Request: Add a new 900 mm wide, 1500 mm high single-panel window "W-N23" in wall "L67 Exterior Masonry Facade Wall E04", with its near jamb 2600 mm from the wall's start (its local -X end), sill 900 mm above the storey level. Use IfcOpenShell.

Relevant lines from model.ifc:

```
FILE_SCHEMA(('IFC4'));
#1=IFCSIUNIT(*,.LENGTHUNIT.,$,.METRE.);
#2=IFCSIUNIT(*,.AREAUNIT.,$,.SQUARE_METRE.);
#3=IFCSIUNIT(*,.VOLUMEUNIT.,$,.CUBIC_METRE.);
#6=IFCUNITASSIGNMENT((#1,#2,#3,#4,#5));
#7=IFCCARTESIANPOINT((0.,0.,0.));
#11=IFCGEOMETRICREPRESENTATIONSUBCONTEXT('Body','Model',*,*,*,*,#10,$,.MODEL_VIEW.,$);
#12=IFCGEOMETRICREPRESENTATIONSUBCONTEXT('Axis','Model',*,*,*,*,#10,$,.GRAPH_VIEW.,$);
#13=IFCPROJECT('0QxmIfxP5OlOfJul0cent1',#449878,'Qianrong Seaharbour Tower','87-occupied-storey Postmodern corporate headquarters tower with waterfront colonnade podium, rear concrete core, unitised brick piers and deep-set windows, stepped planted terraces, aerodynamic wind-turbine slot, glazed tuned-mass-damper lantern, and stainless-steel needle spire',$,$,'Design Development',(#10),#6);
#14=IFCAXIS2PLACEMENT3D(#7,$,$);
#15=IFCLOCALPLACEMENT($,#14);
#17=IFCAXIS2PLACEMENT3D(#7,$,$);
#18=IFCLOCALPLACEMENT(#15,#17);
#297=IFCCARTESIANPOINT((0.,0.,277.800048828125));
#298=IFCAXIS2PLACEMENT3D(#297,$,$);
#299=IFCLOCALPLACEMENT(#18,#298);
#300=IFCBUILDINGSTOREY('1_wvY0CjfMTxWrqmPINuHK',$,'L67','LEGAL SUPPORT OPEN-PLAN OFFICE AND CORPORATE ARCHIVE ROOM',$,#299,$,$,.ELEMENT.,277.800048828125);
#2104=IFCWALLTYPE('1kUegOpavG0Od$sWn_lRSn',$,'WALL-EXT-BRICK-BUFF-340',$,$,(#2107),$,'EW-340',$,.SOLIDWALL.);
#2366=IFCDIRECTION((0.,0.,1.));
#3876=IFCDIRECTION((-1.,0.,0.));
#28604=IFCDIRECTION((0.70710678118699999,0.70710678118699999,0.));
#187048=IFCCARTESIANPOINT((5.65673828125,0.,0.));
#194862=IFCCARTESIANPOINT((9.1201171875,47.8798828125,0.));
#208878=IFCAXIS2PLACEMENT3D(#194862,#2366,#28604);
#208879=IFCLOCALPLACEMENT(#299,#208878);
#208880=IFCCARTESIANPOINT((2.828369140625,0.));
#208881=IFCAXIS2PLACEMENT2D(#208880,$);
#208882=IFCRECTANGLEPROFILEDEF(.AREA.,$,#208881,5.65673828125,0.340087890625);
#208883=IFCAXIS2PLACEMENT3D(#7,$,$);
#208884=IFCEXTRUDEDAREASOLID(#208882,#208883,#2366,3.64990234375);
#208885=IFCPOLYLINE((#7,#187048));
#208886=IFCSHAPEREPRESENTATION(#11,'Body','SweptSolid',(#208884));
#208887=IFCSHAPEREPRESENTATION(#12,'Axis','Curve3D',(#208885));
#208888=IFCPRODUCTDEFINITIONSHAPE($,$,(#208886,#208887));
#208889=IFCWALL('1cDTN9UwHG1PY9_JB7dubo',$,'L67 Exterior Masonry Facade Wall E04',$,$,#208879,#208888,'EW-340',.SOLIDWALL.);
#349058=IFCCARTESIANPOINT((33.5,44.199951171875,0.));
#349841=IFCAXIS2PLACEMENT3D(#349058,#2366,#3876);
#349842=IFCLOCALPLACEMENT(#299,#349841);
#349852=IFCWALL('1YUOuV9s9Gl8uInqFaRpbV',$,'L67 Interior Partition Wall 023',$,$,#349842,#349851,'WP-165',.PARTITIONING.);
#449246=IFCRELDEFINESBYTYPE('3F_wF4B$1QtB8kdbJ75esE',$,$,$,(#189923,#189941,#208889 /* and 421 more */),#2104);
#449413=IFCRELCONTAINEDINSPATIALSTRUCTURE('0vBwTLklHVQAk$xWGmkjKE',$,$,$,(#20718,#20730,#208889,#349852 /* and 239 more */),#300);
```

```python
import numpy as np
import ifcopenshell
import ifcopenshell.api.feature
import ifcopenshell.api.geometry
import ifcopenshell.api.root
import ifcopenshell.api.spatial
import ifcopenshell.geom
import ifcopenshell.util.element
import ifcopenshell.util.placement
import ifcopenshell.util.representation
import ifcopenshell.util.shape
import ifcopenshell.util.unit

model = ifcopenshell.open("model.ifc")
unit_scale = ifcopenshell.util.unit.calculate_unit_scale(model)
settings = ifcopenshell.geom.settings()


def volume(element):
    """Net volume in cubic metres, openings subtracted."""
    shape = ifcopenshell.geom.create_shape(settings, element)
    return ifcopenshell.util.shape.get_volume(shape.geometry)


wall = model.by_id(208889)
storey = ifcopenshell.util.element.get_container(wall, ifc_class="IfcBuildingStorey")
context = ifcopenshell.util.representation.get_context(model, "Model", "Body", "MODEL_VIEW")
before = volume(wall)

width, height, from_end, sill = 0.9, 1.5, 2.6, 0.9  # metres

# The wall runs along its own X axis, and the end named is its -X end.
wall_shape = ifcopenshell.geom.create_shape(settings, wall)
x, y, z = ifcopenshell.util.shape.get_vertices(wall_shape.geometry).T
start = x.min() + from_end
face, thickness = float(y.min()), float(y.max() - y.min())
wall_matrix = ifcopenshell.util.placement.get_local_placement(wall.ObjectPlacement)
level = ifcopenshell.util.placement.get_local_placement(storey.ObjectPlacement)[2, 3]


def in_wall(x, y):
    """Placement at x, y metres in the wall's axes, at sill height."""
    matrix = wall_matrix.copy()
    matrix[:, 3] = wall_matrix @ np.array([x / unit_scale, y / unit_scale, 0.0, 1.0])
    matrix[2, 3] = level + sill / unit_scale
    return matrix


# Opening: a box that overshoots both wall faces by 50 mm.
opening = ifcopenshell.api.root.create_entity(model, ifc_class="IfcOpeningElement", predefined_type="OPENING")
box = ifcopenshell.api.geometry.add_wall_representation(
    model, context=context, length=width, height=height, thickness=thickness + 0.1
)
ifcopenshell.api.geometry.assign_representation(model, product=opening, representation=box)
ifcopenshell.api.geometry.edit_object_placement(model, product=opening, matrix=in_wall(start, face - 0.05), is_si=False)
ifcopenshell.api.feature.add_feature(model, feature=opening, element=wall)

window = ifcopenshell.api.root.create_entity(model, ifc_class="IfcWindow", name="W-N23", predefined_type="WINDOW")
window.OverallWidth, window.OverallHeight = width / unit_scale, height / unit_scale
window.PartitioningType = "SINGLE_PANEL"
body = ifcopenshell.api.geometry.add_window_representation(
    model,
    context=context,
    overall_width=window.OverallWidth,
    overall_height=window.OverallHeight,
    partition_type="SINGLE_PANEL",
)
ifcopenshell.api.geometry.assign_representation(model, product=window, representation=body)
ifcopenshell.api.spatial.assign_container(model, products=[window], relating_structure=storey)
ifcopenshell.api.feature.add_filling(model, opening=opening, element=window)

# Centre the window in the wall's thickness.
ifcopenshell.api.geometry.edit_object_placement(model, product=window, matrix=in_wall(start, face), is_si=False)
window_shape = ifcopenshell.geom.create_shape(settings, window)
depth = ifcopenshell.util.shape.get_vertices(window_shape.geometry)[:, 1]
offset = face + thickness / 2 - (depth.min() + depth.max()) / 2
ifcopenshell.api.geometry.edit_object_placement(model, product=window, matrix=in_wall(start, offset), is_si=False)

after = volume(wall)

print(f"wall volume {before:.3f} -> {after:.3f} m3")

model.write("model_v2.ifc")
```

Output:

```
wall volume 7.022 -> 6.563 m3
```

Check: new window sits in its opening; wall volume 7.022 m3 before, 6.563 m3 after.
